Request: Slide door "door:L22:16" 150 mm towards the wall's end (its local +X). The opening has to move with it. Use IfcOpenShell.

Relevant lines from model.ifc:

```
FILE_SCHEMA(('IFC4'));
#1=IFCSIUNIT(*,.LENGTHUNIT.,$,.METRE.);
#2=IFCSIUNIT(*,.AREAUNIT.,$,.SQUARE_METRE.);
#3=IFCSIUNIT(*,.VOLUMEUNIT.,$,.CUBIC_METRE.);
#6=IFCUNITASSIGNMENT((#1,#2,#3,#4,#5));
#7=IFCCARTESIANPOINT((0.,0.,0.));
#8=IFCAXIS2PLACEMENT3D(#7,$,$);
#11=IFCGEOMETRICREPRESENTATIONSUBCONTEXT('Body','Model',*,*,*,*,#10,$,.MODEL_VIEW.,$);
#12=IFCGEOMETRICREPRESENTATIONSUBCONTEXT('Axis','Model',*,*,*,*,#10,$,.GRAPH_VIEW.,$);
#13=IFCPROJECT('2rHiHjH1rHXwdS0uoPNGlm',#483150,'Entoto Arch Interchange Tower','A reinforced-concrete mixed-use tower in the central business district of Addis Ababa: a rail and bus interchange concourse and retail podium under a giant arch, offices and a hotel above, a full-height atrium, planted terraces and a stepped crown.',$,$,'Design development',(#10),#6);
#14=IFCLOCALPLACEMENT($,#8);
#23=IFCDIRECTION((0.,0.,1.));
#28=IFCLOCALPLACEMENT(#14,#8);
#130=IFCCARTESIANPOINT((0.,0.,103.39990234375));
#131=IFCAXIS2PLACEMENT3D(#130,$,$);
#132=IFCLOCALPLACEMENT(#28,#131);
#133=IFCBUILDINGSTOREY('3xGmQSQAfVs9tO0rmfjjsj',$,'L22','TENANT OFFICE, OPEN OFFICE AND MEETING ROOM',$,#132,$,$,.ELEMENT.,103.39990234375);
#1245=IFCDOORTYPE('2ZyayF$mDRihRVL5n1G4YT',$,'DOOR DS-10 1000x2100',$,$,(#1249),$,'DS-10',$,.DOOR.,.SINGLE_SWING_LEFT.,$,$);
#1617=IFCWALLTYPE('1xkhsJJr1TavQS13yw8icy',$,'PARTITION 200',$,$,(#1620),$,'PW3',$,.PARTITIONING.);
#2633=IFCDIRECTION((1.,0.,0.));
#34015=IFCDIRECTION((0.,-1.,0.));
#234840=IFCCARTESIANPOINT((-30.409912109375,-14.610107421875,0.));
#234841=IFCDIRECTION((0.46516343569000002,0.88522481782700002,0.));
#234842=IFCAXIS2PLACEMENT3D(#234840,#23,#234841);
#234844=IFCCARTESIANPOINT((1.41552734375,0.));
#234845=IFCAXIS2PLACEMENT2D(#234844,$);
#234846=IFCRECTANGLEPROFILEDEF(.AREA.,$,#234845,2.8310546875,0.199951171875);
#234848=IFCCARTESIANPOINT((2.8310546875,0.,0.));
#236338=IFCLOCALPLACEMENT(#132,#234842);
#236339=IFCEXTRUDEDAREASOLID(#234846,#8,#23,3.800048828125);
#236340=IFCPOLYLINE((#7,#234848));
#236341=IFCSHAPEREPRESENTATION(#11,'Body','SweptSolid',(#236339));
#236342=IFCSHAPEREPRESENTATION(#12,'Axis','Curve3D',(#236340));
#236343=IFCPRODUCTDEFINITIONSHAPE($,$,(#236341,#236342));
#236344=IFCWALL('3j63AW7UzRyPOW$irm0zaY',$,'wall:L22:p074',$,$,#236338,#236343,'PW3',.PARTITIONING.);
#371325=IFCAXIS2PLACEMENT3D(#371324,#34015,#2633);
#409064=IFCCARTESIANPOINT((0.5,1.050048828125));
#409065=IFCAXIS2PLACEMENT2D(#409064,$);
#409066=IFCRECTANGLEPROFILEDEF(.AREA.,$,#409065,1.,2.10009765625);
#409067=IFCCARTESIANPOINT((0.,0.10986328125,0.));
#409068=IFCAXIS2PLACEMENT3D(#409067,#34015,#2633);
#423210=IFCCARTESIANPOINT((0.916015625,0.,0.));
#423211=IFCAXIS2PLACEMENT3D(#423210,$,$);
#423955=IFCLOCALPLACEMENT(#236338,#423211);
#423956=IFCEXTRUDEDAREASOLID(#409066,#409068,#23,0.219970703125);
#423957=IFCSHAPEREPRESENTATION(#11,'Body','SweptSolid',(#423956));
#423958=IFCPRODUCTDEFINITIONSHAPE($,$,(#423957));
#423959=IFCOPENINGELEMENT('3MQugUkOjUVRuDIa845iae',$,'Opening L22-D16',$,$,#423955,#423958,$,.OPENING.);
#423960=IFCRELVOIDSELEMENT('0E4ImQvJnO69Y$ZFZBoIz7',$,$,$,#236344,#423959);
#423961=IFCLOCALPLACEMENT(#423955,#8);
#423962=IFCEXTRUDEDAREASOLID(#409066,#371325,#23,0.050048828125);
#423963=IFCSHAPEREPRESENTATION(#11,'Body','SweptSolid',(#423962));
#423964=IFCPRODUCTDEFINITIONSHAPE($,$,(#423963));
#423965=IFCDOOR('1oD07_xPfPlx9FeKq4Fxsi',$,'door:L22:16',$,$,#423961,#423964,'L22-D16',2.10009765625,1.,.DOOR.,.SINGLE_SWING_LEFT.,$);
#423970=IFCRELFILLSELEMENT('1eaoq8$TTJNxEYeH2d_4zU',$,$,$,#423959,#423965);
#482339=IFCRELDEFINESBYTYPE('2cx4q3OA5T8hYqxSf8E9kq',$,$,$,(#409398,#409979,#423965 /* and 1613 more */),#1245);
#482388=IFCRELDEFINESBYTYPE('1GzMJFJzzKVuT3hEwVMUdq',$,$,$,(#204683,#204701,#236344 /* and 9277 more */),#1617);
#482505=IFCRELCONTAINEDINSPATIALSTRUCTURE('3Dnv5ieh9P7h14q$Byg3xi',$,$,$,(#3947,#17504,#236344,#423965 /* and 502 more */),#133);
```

```python
import ifcopenshell
import ifcopenshell.api.geometry
import ifcopenshell.util.placement
import ifcopenshell.util.unit

model = ifcopenshell.open("model.ifc")
unit_scale = ifcopenshell.util.unit.calculate_unit_scale(model)

door = model.by_guid("1oD07_xPfPlx9FeKq4Fxsi")
opening = door.FillsVoids[0].RelatingOpeningElement
wall = opening.VoidsElements[0].RelatingBuildingElement

wall_matrix = ifcopenshell.util.placement.get_local_placement(wall.ObjectPlacement)
shift = wall_matrix[:3, 0] * 0.15 / unit_scale
before = ifcopenshell.util.placement.get_local_placement(door.ObjectPlacement)[:3, 3].copy()

# The door is placed relative to its opening, so it follows when the opening moves.
matrix = ifcopenshell.util.placement.get_local_placement(opening.ObjectPlacement)
matrix[:3, 3] += shift
ifcopenshell.api.geometry.edit_object_placement(
    model, product=opening, matrix=matrix, is_si=False, should_transform_children=True
)

after = ifcopenshell.util.placement.get_local_placement(door.ObjectPlacement)[:3, 3]
print("door moved by", (after - before).round(3) + 0.0)

model.write("model_edited.ifc")
```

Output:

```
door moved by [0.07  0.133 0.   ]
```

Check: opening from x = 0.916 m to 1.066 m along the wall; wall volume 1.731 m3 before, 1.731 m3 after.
